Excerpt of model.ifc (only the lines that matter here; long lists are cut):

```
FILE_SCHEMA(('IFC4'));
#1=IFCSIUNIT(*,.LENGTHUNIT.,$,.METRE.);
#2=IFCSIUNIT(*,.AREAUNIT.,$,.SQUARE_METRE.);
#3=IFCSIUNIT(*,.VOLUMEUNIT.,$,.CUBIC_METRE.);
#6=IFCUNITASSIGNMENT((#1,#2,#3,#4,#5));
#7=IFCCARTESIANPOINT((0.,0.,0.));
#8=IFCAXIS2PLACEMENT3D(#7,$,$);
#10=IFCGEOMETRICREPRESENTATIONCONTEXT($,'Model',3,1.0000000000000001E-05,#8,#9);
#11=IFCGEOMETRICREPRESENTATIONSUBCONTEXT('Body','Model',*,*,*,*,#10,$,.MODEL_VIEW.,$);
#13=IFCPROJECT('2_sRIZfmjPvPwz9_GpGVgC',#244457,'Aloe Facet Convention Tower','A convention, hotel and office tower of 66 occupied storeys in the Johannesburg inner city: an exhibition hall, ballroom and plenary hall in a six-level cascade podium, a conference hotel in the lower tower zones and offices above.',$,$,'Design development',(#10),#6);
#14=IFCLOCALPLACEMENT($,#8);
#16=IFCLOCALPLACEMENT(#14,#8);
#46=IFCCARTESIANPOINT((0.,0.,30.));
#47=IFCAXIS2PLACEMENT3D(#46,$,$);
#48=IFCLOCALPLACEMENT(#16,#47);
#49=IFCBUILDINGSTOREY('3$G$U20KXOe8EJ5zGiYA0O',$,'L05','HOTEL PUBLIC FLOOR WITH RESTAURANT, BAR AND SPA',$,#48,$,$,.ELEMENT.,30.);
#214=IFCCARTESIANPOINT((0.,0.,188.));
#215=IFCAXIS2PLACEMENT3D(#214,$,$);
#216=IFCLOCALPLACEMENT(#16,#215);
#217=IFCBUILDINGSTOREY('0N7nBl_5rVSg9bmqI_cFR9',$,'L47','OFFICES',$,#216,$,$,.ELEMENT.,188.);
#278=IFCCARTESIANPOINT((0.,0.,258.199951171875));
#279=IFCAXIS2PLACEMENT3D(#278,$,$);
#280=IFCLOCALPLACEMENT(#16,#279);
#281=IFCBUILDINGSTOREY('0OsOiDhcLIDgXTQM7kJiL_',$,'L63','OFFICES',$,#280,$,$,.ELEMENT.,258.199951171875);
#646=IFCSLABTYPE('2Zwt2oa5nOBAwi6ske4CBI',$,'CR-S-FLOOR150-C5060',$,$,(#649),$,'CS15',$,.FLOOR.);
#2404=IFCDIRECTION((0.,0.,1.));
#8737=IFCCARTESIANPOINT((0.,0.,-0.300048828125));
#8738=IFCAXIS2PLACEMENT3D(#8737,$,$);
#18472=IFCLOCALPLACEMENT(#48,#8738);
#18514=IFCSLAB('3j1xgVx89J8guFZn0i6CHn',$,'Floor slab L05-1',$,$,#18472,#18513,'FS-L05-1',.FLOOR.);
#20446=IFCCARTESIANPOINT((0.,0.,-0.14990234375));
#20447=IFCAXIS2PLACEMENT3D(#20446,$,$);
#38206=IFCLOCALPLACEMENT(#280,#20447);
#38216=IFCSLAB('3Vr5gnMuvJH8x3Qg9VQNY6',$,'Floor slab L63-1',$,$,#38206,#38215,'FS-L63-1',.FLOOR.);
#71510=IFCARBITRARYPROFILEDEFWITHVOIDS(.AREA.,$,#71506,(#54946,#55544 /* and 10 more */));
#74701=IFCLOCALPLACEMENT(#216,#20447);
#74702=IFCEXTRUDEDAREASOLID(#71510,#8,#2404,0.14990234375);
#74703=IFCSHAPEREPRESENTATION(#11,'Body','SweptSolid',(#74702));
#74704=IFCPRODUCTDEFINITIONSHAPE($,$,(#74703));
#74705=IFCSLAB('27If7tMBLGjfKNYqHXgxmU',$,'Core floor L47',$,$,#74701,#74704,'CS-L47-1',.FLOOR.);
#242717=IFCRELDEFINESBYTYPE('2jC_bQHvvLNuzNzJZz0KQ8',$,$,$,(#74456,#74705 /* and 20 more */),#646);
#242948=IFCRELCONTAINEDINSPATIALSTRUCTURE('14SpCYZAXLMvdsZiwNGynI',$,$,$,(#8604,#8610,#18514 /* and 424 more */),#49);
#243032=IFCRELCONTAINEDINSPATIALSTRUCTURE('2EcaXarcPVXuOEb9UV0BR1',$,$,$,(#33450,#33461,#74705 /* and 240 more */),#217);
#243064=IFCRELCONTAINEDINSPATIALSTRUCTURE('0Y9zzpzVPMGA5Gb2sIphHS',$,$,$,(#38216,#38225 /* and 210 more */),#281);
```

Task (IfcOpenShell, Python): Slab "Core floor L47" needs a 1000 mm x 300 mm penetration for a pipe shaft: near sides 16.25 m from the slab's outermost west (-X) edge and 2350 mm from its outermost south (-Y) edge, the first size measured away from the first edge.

```python
import numpy as np
import ifcopenshell
import ifcopenshell.api.feature
import ifcopenshell.api.geometry
import ifcopenshell.api.root
import ifcopenshell.geom
import ifcopenshell.util.placement
import ifcopenshell.util.representation
import ifcopenshell.util.shape
import ifcopenshell.util.unit

model = ifcopenshell.open("model.ifc")
unit_scale = ifcopenshell.util.unit.calculate_unit_scale(model)
settings = ifcopenshell.geom.settings()


def volume(element):
    """Net volume in cubic metres, openings subtracted."""
    shape = ifcopenshell.geom.create_shape(settings, element)
    return ifcopenshell.util.shape.get_volume(shape.geometry)


slab = model.by_guid("27If7tMBLGjfKNYqHXgxmU")
before = volume(slab)

# Extent in the slab's own axes, in metres. The edges named are its -X and -Y sides.
slab_shape = ifcopenshell.geom.create_shape(settings, slab)
vertices = ifcopenshell.util.shape.get_vertices(slab_shape.geometry)
x_min, y_min, bottom = vertices.min(axis=0)
top = vertices[:, 2].max()

opening = ifcopenshell.api.root.create_entity(model, ifc_class="IfcOpeningElement", name="Pipe shaft opening", predefined_type="OPENING")
context = ifcopenshell.util.representation.get_context(model, "Model", "Body", "MODEL_VIEW")
width, depth = 1, 0.3
outline = [(0.0, 0.0), (width, 0.0), (width, depth), (0.0, depth), (0.0, 0.0)]
# Overshoot both faces by 50 mm so the cut is clean.
shape = ifcopenshell.api.geometry.add_slab_representation(
    model, context=context, depth=top - bottom + 0.1, polyline=outline
)
ifcopenshell.api.geometry.assign_representation(model, product=opening, representation=shape)

matrix = ifcopenshell.util.placement.get_local_placement(slab.ObjectPlacement)
matrix[:, 3] = matrix @ np.append(np.array([x_min + 16.25, y_min + 2.35, bottom - 0.05]) / unit_scale, 1.0)
ifcopenshell.api.geometry.edit_object_placement(model, product=opening, matrix=matrix, is_si=False)
ifcopenshell.api.feature.add_feature(model, feature=opening, element=slab)

after = volume(slab)

print(f"slab volume {before:.3f} -> {after:.3f} m3")

model.write("model_updated.ifc")
```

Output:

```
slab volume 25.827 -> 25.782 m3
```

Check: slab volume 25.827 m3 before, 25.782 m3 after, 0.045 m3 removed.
